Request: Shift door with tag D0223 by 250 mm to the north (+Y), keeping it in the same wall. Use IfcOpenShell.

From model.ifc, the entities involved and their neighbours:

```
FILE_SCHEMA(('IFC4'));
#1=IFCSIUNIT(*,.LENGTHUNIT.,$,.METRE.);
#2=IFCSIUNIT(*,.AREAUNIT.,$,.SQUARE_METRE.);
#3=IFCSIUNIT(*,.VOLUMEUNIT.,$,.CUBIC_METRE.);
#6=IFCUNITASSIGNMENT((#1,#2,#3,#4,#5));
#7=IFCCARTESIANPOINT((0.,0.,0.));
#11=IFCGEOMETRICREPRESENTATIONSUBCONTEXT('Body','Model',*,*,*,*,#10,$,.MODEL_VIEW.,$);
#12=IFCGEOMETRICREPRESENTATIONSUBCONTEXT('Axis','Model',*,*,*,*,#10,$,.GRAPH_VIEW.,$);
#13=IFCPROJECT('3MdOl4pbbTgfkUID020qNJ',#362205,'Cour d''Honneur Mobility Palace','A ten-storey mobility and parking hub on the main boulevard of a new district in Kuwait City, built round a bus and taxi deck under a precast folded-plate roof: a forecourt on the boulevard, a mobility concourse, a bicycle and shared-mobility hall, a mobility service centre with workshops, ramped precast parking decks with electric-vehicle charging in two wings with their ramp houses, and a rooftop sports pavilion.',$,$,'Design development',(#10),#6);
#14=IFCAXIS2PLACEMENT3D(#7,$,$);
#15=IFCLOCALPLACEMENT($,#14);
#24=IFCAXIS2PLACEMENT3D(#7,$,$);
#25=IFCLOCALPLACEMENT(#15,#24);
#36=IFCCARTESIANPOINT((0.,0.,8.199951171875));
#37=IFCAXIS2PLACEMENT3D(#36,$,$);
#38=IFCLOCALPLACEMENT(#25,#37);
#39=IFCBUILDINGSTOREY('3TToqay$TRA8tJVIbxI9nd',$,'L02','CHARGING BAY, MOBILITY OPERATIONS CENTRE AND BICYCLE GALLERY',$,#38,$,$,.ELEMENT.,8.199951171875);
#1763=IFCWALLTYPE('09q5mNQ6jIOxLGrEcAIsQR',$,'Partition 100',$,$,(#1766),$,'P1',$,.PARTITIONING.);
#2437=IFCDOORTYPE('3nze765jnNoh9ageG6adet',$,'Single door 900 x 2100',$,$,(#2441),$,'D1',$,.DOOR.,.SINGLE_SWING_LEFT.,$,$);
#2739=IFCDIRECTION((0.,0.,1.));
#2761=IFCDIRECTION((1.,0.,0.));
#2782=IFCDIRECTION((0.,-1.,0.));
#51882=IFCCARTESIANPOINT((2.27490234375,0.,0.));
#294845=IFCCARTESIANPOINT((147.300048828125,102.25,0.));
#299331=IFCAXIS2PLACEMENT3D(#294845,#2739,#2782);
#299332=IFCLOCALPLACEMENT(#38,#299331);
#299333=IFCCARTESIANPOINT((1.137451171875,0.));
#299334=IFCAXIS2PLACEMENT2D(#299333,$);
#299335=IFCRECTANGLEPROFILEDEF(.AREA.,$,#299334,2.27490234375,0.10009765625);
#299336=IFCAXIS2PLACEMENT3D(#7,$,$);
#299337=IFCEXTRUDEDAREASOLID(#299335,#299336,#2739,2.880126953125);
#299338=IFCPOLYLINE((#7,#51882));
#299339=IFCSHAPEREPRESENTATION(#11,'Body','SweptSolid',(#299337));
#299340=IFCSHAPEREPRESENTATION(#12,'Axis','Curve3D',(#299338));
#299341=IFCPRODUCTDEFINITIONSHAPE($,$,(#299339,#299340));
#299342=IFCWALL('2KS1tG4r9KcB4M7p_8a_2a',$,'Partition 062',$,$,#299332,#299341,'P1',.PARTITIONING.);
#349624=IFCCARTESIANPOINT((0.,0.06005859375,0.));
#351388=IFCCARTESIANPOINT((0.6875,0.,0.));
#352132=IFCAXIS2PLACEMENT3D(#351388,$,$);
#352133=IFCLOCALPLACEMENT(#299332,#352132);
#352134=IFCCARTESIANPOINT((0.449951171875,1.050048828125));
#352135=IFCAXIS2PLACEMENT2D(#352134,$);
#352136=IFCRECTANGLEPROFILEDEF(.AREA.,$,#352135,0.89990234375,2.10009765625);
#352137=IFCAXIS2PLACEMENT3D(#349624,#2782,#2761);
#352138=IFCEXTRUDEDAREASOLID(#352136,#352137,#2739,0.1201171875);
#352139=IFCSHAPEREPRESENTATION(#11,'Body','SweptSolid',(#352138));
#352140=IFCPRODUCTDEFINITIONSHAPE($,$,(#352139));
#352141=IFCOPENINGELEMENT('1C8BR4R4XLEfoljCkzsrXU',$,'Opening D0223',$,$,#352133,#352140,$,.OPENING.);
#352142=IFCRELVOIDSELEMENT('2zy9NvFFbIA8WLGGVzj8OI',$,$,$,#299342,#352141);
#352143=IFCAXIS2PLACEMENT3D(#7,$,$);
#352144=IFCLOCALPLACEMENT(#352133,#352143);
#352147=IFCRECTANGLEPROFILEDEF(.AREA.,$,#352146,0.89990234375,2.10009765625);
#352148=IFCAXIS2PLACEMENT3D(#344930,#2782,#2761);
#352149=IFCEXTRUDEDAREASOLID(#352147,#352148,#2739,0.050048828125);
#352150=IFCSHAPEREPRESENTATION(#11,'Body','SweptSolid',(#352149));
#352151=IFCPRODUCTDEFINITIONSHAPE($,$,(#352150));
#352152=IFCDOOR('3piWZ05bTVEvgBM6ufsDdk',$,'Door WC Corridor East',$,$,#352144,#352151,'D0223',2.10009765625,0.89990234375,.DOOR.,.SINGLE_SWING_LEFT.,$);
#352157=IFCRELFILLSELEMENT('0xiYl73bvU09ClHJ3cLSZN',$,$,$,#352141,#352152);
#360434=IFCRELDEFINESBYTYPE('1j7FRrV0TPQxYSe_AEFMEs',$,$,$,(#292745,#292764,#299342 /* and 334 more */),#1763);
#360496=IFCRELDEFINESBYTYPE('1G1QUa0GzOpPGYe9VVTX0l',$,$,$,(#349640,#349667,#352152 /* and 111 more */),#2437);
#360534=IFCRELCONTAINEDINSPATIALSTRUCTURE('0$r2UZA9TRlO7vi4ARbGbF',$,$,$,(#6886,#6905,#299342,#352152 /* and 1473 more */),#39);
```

```python
import ifcopenshell
import ifcopenshell.api.geometry
import ifcopenshell.util.placement
import ifcopenshell.util.unit

model = ifcopenshell.open("model.ifc")
unit_scale = ifcopenshell.util.unit.calculate_unit_scale(model)

door = model.by_guid("3piWZ05bTVEvgBM6ufsDdk")
opening = door.FillsVoids[0].RelatingOpeningElement
wall = opening.VoidsElements[0].RelatingBuildingElement

wall_matrix = ifcopenshell.util.placement.get_local_placement(wall.ObjectPlacement)
shift = wall_matrix[:3, 0] * -0.25 / unit_scale
before = ifcopenshell.util.placement.get_local_placement(door.ObjectPlacement)[:3, 3].copy()

# The door is placed relative to its opening, so it follows when the opening moves.
matrix = ifcopenshell.util.placement.get_local_placement(opening.ObjectPlacement)
matrix[:3, 3] += shift
ifcopenshell.api.geometry.edit_object_placement(
    model, product=opening, matrix=matrix, is_si=False, should_transform_children=True
)

after = ifcopenshell.util.placement.get_local_placement(door.ObjectPlacement)[:3, 3]
print("door moved by", (after - before).round(3) + 0.0)

model.write("model_edited.ifc")
```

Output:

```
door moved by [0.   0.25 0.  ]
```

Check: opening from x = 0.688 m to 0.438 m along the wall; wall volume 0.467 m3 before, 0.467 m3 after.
